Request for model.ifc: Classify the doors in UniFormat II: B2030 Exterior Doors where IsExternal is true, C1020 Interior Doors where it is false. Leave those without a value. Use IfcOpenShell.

First a look at what the model holds.

```python
import ifcopenshell
import ifcopenshell.util.element

model = ifcopenshell.open("model.ifc")
print(model.schema)
print("classifications:", [c.Name for c in model.by_type("IfcClassification")])
values = [ifcopenshell.util.element.get_pset(e, "Pset_DoorCommon", "IsExternal") for e in model.by_type("IfcDoor")]
for value in (True, False, None):
    print("IsExternal", value, values.count(value))
```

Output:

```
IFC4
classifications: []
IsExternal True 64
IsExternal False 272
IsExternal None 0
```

```python
import ifcopenshell
import ifcopenshell.api.classification
import ifcopenshell.util.element

model = ifcopenshell.open("model.ifc")

system = ifcopenshell.api.classification.add_classification(model, classification="UniFormat II")

doors = model.by_type("IfcDoor")
external = {e: ifcopenshell.util.element.get_pset(e, "Pset_DoorCommon", "IsExternal") for e in doors}
for flag, code, name in ((True, "B2030", "Exterior Doors"), (False, "C1020", "Interior Doors")):
    products = [e for e in doors if external[e] is flag]
    ifcopenshell.api.classification.add_reference(
        model, products=products, classification=system, identification=code, name=name
    )
    print(code, len(products))

model.write("model_v2.ifc")
```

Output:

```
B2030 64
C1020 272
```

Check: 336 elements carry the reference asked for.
